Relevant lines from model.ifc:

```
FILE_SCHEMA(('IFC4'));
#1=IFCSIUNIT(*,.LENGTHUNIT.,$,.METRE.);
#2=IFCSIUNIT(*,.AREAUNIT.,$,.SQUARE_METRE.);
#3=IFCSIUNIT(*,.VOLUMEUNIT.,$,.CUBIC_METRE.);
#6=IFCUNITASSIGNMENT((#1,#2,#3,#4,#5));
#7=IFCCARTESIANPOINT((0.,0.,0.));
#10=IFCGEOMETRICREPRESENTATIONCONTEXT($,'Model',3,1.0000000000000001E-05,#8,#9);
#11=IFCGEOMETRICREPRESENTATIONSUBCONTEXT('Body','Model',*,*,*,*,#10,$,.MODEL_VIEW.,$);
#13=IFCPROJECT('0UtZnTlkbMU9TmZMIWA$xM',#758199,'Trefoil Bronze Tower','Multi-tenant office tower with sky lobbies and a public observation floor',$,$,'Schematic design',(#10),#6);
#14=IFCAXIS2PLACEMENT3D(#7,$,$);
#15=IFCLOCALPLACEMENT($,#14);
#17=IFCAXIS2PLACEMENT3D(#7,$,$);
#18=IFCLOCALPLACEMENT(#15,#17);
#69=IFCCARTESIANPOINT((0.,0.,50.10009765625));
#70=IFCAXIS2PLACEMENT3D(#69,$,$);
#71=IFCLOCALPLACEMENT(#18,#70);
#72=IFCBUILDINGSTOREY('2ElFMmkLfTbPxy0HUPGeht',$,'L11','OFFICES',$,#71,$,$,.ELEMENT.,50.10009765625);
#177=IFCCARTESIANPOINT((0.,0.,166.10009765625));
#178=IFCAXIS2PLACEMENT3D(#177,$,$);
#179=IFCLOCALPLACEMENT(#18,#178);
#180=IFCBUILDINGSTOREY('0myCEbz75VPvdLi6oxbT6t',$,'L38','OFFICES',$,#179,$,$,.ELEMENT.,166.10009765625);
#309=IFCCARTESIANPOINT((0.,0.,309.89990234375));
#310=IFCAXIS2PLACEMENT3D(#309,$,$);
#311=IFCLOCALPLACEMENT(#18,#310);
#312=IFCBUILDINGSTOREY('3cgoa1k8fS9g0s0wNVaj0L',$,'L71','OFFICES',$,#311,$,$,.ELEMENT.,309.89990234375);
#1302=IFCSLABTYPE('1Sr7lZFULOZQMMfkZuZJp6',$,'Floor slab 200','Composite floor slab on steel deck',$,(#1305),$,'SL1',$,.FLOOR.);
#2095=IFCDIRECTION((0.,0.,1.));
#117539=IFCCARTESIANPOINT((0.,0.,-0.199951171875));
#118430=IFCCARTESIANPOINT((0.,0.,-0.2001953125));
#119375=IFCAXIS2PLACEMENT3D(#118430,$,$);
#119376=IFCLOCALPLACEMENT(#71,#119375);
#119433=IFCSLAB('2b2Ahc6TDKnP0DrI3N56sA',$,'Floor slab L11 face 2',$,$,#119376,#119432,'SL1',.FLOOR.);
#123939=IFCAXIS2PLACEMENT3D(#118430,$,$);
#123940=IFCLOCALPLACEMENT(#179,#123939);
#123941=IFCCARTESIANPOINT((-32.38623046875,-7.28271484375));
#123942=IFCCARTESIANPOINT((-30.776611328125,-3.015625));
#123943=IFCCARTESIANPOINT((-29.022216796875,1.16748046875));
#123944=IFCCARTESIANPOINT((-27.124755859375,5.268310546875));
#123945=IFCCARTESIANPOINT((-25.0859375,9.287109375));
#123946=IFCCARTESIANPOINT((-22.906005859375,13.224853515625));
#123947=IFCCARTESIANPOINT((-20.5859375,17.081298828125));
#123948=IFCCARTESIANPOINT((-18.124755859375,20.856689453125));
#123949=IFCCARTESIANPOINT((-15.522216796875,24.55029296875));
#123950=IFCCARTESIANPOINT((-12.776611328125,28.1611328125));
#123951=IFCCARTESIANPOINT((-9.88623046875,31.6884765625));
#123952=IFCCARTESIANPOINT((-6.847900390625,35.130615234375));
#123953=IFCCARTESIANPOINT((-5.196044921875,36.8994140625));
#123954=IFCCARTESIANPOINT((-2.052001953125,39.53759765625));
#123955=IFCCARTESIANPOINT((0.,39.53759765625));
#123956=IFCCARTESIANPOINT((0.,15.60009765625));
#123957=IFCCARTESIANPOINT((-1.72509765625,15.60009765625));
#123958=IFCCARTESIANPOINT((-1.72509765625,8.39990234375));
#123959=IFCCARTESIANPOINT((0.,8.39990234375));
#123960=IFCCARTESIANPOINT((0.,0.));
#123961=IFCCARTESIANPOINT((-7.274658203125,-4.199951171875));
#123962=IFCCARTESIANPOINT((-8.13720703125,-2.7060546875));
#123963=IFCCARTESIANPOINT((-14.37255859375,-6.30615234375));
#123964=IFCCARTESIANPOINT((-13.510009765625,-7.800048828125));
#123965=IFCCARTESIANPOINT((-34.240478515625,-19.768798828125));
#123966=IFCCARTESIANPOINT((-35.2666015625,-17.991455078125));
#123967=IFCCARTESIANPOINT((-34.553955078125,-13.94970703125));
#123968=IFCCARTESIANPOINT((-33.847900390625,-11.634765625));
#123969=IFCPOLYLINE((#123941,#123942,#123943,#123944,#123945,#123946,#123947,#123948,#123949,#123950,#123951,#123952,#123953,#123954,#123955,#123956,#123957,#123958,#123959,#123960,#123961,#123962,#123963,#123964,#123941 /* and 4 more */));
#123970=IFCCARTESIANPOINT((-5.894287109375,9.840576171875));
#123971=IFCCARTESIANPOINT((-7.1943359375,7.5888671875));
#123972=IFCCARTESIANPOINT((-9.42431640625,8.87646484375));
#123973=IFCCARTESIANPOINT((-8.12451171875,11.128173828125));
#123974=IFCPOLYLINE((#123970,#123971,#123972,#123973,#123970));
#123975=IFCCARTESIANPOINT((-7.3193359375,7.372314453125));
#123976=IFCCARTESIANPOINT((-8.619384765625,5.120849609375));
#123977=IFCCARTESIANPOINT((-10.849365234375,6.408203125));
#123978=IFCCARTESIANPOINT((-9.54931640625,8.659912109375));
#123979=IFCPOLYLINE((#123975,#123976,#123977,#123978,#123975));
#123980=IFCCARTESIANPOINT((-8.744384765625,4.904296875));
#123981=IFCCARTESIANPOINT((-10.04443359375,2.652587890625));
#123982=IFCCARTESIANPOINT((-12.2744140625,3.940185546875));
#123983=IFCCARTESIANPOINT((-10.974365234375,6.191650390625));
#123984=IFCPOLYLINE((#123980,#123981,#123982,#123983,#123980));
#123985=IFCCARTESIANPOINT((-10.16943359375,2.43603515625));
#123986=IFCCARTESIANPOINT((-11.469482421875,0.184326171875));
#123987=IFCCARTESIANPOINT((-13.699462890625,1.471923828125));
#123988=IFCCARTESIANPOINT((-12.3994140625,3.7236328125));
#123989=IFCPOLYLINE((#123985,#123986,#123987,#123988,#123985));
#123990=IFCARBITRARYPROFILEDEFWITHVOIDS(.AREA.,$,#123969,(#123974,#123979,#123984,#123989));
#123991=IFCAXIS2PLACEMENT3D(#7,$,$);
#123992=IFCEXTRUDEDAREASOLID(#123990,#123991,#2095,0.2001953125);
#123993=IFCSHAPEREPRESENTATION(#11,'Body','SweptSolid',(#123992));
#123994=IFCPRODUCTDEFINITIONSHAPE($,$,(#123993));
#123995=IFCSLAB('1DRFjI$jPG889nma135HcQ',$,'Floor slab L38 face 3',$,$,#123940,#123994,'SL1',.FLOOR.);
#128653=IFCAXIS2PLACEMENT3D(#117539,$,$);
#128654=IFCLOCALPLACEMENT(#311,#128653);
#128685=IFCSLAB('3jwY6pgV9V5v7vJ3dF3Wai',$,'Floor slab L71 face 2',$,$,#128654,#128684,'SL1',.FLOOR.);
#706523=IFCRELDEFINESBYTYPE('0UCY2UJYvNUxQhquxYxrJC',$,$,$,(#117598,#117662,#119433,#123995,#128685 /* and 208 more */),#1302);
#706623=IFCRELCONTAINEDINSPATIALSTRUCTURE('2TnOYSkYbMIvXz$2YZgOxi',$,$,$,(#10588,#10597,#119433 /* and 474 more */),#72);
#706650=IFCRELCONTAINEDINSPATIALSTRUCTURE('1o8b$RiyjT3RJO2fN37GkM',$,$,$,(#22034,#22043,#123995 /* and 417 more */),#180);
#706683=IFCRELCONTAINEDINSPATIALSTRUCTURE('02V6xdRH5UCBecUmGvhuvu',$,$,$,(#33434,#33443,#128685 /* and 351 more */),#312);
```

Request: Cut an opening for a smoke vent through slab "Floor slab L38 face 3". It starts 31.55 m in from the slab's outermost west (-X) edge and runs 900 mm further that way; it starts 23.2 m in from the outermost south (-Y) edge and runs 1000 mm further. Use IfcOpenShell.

```python
import numpy as np
import ifcopenshell
import ifcopenshell.api.feature
import ifcopenshell.api.geometry
import ifcopenshell.api.root
import ifcopenshell.geom
import ifcopenshell.util.placement
import ifcopenshell.util.representation
import ifcopenshell.util.shape
import ifcopenshell.util.unit

model = ifcopenshell.open("model.ifc")
unit_scale = ifcopenshell.util.unit.calculate_unit_scale(model)
settings = ifcopenshell.geom.settings()


def volume(element):
    """Net volume in cubic metres, openings subtracted."""
    shape = ifcopenshell.geom.create_shape(settings, element)
    return ifcopenshell.util.shape.get_volume(shape.geometry)


slab = model.by_guid("1DRFjI$jPG889nma135HcQ")
before = volume(slab)

# Extent in the slab's own axes, in metres. The edges named are its -X and -Y sides.
slab_shape = ifcopenshell.geom.create_shape(settings, slab)
vertices = ifcopenshell.util.shape.get_vertices(slab_shape.geometry)
x_min, y_min, bottom = vertices.min(axis=0)
top = vertices[:, 2].max()

opening = ifcopenshell.api.root.create_entity(model, ifc_class="IfcOpeningElement", name="Smoke vent opening", predefined_type="OPENING")
context = ifcopenshell.util.representation.get_context(model, "Model", "Body", "MODEL_VIEW")
width, depth = 0.9, 1
outline = [(0.0, 0.0), (width, 0.0), (width, depth), (0.0, depth), (0.0, 0.0)]
# Overshoot both faces by 50 mm so the cut is clean.
shape = ifcopenshell.api.geometry.add_slab_representation(
    model, context=context, depth=top - bottom + 0.1, polyline=outline
)
ifcopenshell.api.geometry.assign_representation(model, product=opening, representation=shape)

matrix = ifcopenshell.util.placement.get_local_placement(slab.ObjectPlacement)
matrix[:, 3] = matrix @ np.append(np.array([x_min + 31.55, y_min + 23.2, bottom - 0.05]) / unit_scale, 1.0)
ifcopenshell.api.geometry.edit_object_placement(model, product=opening, matrix=matrix, is_si=False)
ifcopenshell.api.feature.add_feature(model, feature=opening, element=slab)

after = volume(slab)

print(f"slab volume {before:.3f} -> {after:.3f} m3")

model.write("model-out.ifc")
```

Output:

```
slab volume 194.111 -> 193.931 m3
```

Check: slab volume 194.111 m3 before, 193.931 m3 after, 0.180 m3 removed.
